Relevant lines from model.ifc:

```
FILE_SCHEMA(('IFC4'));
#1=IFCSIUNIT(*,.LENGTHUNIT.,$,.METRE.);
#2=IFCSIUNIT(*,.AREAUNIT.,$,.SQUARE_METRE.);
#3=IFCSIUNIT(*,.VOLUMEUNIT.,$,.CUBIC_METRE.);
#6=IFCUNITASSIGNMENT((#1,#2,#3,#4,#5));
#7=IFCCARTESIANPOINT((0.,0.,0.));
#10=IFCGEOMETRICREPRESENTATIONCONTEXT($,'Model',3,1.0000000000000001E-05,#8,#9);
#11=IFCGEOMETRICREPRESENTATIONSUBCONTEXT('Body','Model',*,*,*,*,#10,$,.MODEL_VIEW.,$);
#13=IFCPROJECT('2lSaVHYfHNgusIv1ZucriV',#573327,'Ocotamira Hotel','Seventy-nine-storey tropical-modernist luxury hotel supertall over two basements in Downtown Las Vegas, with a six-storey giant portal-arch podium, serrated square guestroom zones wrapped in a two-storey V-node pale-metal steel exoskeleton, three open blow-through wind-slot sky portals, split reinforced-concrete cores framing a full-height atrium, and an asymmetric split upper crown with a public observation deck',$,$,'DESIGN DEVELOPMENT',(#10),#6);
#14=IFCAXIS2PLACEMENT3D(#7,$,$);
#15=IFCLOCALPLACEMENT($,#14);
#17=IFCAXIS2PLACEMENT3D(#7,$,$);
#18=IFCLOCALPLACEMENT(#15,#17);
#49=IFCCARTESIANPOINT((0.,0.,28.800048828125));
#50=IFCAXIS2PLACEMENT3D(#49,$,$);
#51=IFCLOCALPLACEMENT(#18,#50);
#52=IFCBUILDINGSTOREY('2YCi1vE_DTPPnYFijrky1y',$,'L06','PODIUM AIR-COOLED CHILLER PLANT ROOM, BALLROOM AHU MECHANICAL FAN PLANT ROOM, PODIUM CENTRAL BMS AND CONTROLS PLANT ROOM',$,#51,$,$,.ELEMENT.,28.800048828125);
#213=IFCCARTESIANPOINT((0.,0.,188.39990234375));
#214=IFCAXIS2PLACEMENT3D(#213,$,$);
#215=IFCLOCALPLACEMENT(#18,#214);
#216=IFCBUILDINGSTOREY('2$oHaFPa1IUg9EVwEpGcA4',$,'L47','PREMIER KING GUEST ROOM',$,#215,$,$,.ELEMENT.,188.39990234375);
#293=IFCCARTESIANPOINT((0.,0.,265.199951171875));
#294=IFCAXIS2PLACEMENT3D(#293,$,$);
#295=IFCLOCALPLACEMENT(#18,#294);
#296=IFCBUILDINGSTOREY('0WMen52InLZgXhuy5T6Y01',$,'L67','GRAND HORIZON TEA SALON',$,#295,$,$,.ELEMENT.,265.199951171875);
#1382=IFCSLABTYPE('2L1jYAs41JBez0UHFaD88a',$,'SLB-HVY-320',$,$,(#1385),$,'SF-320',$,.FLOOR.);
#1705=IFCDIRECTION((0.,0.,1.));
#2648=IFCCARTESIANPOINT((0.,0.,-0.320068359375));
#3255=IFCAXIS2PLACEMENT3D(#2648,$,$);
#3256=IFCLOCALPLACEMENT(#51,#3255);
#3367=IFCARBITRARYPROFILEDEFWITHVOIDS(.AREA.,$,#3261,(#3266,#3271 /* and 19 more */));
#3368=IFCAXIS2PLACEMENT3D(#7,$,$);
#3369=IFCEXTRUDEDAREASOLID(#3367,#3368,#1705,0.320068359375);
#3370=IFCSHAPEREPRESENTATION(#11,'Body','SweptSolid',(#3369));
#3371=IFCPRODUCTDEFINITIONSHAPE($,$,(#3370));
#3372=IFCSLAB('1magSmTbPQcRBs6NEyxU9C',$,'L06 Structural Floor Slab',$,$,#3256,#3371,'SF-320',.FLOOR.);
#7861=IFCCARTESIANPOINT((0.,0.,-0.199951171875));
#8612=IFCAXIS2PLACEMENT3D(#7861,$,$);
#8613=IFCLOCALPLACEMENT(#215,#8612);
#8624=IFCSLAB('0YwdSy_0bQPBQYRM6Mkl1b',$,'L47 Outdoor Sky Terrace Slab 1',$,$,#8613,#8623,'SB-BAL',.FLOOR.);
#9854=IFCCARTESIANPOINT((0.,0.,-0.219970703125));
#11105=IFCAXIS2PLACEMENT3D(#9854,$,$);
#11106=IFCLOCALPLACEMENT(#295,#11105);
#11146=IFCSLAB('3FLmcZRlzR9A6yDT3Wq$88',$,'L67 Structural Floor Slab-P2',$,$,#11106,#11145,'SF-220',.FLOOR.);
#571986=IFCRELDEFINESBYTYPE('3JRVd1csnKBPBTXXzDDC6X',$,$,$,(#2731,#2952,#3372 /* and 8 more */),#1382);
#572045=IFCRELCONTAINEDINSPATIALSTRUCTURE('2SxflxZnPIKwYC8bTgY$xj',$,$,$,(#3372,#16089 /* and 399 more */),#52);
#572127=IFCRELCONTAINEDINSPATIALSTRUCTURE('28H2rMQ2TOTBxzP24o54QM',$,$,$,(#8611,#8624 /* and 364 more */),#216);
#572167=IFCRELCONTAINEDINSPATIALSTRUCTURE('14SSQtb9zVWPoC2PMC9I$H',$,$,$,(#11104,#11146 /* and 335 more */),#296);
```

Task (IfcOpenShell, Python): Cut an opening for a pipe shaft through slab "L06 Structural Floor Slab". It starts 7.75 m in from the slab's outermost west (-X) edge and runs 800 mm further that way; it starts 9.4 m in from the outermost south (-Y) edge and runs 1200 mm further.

```python
import numpy as np
import ifcopenshell
import ifcopenshell.api.feature
import ifcopenshell.api.geometry
import ifcopenshell.api.root
import ifcopenshell.geom
import ifcopenshell.util.placement
import ifcopenshell.util.representation
import ifcopenshell.util.shape
import ifcopenshell.util.unit

model = ifcopenshell.open("model.ifc")
unit_scale = ifcopenshell.util.unit.calculate_unit_scale(model)
settings = ifcopenshell.geom.settings()


def volume(element):
    """Net volume in cubic metres, openings subtracted."""
    shape = ifcopenshell.geom.create_shape(settings, element)
    return ifcopenshell.util.shape.get_volume(shape.geometry)


slab = model.by_guid("1magSmTbPQcRBs6NEyxU9C")
before = volume(slab)

# Extent in the slab's own axes, in metres. The edges named are its -X and -Y sides.
slab_shape = ifcopenshell.geom.create_shape(settings, slab)
vertices = ifcopenshell.util.shape.get_vertices(slab_shape.geometry)
x_min, y_min, bottom = vertices.min(axis=0)
top = vertices[:, 2].max()

opening = ifcopenshell.api.root.create_entity(model, ifc_class="IfcOpeningElement", name="Pipe shaft opening", predefined_type="OPENING")
context = ifcopenshell.util.representation.get_context(model, "Model", "Body", "MODEL_VIEW")
width, depth = 0.8, 1.2
outline = [(0.0, 0.0), (width, 0.0), (width, depth), (0.0, depth), (0.0, 0.0)]
# Overshoot both faces by 50 mm so the cut is clean.
shape = ifcopenshell.api.geometry.add_slab_representation(
    model, context=context, depth=top - bottom + 0.1, polyline=outline
)
ifcopenshell.api.geometry.assign_representation(model, product=opening, representation=shape)

matrix = ifcopenshell.util.placement.get_local_placement(slab.ObjectPlacement)
matrix[:, 3] = matrix @ np.append(np.array([x_min + 7.75, y_min + 9.4, bottom - 0.05]) / unit_scale, 1.0)
ifcopenshell.api.geometry.edit_object_placement(model, product=opening, matrix=matrix, is_si=False)
ifcopenshell.api.feature.add_feature(model, feature=opening, element=slab)

after = volume(slab)

print(f"slab volume {before:.3f} -> {after:.3f} m3")

model.write("model_updated.ifc")
```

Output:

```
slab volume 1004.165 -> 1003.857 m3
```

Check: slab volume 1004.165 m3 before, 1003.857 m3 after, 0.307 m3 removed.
